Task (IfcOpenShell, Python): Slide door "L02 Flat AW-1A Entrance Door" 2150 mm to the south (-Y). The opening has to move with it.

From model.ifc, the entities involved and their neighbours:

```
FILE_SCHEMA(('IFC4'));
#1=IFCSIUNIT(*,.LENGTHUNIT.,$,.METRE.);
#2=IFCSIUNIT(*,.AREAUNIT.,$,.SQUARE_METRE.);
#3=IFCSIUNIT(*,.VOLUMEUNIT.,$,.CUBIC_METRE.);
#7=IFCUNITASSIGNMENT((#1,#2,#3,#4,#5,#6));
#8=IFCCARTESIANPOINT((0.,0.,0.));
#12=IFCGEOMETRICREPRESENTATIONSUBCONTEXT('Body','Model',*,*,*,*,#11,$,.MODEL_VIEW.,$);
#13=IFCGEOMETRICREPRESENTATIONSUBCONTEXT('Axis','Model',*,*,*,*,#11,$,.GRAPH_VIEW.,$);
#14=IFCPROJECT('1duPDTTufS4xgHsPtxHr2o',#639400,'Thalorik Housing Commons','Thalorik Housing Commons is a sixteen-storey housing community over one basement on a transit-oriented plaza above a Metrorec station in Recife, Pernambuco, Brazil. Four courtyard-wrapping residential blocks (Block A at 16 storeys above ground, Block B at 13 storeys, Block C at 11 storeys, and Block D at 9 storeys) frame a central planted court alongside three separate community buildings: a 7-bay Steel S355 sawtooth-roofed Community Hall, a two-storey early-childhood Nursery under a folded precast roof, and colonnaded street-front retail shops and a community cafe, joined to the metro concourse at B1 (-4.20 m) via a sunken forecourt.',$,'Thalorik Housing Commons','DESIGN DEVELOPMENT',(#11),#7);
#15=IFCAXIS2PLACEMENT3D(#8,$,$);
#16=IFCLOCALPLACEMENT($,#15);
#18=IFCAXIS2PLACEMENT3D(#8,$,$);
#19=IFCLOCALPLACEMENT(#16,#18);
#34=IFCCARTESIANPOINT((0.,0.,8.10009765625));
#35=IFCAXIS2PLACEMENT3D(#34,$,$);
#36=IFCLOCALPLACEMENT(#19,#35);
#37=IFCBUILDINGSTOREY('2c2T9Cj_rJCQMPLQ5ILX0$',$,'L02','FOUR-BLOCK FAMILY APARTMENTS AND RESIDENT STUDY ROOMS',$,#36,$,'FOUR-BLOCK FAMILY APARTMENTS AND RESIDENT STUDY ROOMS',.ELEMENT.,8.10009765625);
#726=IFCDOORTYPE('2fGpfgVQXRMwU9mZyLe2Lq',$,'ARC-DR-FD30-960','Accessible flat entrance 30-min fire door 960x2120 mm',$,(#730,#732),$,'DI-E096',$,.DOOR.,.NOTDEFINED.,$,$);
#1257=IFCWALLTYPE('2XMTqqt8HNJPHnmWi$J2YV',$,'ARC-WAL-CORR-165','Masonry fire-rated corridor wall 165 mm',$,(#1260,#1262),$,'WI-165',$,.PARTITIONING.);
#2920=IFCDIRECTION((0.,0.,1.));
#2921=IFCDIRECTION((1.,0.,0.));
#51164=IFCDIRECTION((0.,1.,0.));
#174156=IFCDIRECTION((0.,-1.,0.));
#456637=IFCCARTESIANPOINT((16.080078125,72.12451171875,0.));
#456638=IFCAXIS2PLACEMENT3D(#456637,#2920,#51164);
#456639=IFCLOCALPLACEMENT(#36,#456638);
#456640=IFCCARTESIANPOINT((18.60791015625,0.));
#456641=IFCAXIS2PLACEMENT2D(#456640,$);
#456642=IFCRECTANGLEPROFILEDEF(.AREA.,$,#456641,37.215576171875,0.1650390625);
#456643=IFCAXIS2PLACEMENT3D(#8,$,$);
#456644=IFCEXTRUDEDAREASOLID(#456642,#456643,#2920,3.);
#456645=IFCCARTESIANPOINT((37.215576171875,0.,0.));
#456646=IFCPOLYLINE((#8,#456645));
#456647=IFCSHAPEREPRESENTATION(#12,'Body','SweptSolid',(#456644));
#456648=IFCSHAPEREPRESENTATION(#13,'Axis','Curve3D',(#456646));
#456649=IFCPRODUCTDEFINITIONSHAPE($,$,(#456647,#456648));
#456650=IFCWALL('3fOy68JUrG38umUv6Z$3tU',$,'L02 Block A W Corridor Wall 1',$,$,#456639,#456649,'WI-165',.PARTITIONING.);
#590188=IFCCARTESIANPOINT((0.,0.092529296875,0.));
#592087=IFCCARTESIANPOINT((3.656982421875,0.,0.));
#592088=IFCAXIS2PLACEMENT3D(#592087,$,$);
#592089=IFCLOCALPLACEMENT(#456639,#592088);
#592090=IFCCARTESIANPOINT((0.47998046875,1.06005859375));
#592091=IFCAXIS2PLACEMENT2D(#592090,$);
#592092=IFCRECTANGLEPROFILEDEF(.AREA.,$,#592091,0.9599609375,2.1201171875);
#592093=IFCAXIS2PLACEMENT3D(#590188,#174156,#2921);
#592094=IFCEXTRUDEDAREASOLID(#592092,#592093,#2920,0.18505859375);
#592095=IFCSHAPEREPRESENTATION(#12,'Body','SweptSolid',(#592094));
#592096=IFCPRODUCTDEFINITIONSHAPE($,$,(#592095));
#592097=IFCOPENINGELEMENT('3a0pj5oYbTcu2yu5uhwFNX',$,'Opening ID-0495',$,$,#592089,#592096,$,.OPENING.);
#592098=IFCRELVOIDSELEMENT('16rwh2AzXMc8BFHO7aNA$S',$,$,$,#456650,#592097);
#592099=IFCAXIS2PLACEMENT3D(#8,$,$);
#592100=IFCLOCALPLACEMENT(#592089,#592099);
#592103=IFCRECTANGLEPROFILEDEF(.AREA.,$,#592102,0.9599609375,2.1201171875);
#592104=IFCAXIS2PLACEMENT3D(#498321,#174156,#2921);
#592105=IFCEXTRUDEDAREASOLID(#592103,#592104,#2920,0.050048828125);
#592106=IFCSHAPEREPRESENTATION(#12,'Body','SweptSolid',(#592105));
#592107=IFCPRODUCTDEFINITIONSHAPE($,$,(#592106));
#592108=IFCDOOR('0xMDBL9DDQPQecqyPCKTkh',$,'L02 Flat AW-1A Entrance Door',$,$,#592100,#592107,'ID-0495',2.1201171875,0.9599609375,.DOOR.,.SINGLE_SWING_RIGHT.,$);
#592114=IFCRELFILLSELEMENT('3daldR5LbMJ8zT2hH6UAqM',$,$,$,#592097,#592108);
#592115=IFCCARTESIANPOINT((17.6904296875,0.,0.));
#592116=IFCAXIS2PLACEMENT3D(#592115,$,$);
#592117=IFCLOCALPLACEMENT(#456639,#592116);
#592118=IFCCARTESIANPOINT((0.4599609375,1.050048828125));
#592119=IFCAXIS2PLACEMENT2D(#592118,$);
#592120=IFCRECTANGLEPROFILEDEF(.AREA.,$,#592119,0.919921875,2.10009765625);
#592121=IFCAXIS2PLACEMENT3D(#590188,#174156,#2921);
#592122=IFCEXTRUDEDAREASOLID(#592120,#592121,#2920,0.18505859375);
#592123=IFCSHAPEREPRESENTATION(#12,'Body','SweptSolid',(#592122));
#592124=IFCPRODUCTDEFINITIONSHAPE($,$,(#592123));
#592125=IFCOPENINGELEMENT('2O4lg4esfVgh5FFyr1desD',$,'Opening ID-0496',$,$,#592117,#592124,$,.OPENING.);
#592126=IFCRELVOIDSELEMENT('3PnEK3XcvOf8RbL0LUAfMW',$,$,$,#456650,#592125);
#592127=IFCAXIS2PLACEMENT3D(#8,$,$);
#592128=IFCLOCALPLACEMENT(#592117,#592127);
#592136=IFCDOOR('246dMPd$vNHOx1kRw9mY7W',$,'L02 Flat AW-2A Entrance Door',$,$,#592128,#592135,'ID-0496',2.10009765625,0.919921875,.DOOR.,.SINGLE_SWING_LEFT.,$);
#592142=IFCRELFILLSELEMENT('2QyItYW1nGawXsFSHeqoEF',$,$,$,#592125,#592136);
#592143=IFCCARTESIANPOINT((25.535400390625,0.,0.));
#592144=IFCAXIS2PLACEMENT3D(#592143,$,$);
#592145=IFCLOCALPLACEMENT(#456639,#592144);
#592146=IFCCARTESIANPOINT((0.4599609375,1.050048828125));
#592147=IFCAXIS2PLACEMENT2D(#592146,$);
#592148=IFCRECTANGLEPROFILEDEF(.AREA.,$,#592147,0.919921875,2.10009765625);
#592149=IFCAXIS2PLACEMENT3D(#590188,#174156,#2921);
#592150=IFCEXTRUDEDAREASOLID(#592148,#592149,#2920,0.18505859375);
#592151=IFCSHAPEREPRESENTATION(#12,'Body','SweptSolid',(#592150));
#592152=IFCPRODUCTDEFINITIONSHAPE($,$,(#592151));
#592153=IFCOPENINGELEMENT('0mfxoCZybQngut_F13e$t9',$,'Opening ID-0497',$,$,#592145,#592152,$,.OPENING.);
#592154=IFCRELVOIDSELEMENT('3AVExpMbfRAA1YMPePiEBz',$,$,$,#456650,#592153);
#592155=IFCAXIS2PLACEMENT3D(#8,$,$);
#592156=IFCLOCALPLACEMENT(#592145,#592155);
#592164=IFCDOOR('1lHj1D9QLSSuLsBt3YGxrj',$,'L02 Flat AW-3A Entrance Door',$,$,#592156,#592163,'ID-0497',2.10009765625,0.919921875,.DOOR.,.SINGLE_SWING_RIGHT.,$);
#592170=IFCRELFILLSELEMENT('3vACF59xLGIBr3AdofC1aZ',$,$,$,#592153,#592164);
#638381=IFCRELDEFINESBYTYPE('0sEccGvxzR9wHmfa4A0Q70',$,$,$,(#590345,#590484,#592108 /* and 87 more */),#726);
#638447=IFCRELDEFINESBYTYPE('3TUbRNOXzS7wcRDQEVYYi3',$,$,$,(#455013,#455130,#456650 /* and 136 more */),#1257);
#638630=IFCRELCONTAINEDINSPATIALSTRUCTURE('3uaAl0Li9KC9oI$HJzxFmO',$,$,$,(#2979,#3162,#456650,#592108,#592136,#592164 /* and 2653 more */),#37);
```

```python
import ifcopenshell
import ifcopenshell.api.geometry
import ifcopenshell.util.placement
import ifcopenshell.util.unit

model = ifcopenshell.open("model.ifc")
unit_scale = ifcopenshell.util.unit.calculate_unit_scale(model)

door = model.by_id(592108)
opening = door.FillsVoids[0].RelatingOpeningElement
wall = opening.VoidsElements[0].RelatingBuildingElement

wall_matrix = ifcopenshell.util.placement.get_local_placement(wall.ObjectPlacement)
shift = wall_matrix[:3, 0] * -2.15 / unit_scale
before = ifcopenshell.util.placement.get_local_placement(door.ObjectPlacement)[:3, 3].copy()

# The door is placed relative to its opening, so it follows when the opening moves.
matrix = ifcopenshell.util.placement.get_local_placement(opening.ObjectPlacement)
matrix[:3, 3] += shift
ifcopenshell.api.geometry.edit_object_placement(
    model, product=opening, matrix=matrix, is_si=False, should_transform_children=True
)

after = ifcopenshell.util.placement.get_local_placement(door.ObjectPlacement)[:3, 3]
print("door moved by", (after - before).round(3) + 0.0)

model.write("model_updated.ifc")
```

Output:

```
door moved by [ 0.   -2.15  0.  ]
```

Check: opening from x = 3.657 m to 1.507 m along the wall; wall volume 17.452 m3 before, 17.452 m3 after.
